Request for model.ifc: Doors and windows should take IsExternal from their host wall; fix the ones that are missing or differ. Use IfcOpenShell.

First a look at what the model holds.

```python
import ifcopenshell
import ifcopenshell.util.element

model = ifcopenshell.open("model.ifc")
print(model.schema)
seen = {}
for e in model.by_type("IfcDoor") + model.by_type("IfcWindow"):
    if not e.FillsVoids:
        continue
    host = e.FillsVoids[0].RelatingOpeningElement.VoidsElements[0].RelatingBuildingElement
    own = ifcopenshell.util.element.get_pset(e, f"Pset_{e.is_a()[3:].removesuffix('StandardCase')}Common", "IsExternal")
    wall = ifcopenshell.util.element.get_pset(host, "Pset_WallCommon", "IsExternal")
    seen[e.is_a(), own, wall] = seen.get((e.is_a(), own, wall), 0) + 1
for (cls, own, wall), count in sorted(seen.items(), key=str):
    print(count, cls, "IsExternal:", own, "| host wall:", wall)
```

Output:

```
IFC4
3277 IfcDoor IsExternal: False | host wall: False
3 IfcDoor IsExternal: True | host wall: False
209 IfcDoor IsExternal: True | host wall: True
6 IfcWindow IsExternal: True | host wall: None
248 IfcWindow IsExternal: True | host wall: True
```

```python
import ifcopenshell
import ifcopenshell.api.pset
import ifcopenshell.util.element

model = ifcopenshell.open("model.ifc")

count = 0
for ifc_class, pset_name in (("IfcDoor", "Pset_DoorCommon"), ("IfcWindow", "Pset_WindowCommon")):
    for e in model.by_type(ifc_class):
        if not e.FillsVoids:
            continue
        host = e.FillsVoids[0].RelatingOpeningElement.VoidsElements[0].RelatingBuildingElement
        external = ifcopenshell.util.element.get_pset(host, "Pset_WallCommon", "IsExternal")
        if external is None or ifcopenshell.util.element.get_pset(e, pset_name, "IsExternal") == external:
            continue
        pset = ifcopenshell.api.pset.add_pset(model, product=e, name=pset_name)
        ifcopenshell.api.pset.edit_pset(model, pset=pset, properties={"IsExternal": external})
        count += 1

print(count, "updated")

model.write("model_rev.ifc")
```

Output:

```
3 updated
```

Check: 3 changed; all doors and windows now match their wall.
